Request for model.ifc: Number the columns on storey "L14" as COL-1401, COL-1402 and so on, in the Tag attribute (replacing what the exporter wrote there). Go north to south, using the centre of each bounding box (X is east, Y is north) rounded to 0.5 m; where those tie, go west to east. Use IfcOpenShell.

First a look at what the model holds.

```python
import ifcopenshell
import ifcopenshell.util.element
import ifcopenshell.util.placement

model = ifcopenshell.open("model.ifc")
print(model.schema)
storey = next(s for s in model.by_type("IfcBuildingStorey") if s.Name == "L14")
columns = [e for e in ifcopenshell.util.element.get_decomposition(storey) if e.is_a("IfcColumn")]
for e in sorted(columns, key=lambda e: e.id()):
    origin = ifcopenshell.util.placement.get_local_placement(e.ObjectPlacement)[:3, 3]
    print(e.id(), e.Tag, e.Name, origin.round(2) + 0.0, sep=" | ")
```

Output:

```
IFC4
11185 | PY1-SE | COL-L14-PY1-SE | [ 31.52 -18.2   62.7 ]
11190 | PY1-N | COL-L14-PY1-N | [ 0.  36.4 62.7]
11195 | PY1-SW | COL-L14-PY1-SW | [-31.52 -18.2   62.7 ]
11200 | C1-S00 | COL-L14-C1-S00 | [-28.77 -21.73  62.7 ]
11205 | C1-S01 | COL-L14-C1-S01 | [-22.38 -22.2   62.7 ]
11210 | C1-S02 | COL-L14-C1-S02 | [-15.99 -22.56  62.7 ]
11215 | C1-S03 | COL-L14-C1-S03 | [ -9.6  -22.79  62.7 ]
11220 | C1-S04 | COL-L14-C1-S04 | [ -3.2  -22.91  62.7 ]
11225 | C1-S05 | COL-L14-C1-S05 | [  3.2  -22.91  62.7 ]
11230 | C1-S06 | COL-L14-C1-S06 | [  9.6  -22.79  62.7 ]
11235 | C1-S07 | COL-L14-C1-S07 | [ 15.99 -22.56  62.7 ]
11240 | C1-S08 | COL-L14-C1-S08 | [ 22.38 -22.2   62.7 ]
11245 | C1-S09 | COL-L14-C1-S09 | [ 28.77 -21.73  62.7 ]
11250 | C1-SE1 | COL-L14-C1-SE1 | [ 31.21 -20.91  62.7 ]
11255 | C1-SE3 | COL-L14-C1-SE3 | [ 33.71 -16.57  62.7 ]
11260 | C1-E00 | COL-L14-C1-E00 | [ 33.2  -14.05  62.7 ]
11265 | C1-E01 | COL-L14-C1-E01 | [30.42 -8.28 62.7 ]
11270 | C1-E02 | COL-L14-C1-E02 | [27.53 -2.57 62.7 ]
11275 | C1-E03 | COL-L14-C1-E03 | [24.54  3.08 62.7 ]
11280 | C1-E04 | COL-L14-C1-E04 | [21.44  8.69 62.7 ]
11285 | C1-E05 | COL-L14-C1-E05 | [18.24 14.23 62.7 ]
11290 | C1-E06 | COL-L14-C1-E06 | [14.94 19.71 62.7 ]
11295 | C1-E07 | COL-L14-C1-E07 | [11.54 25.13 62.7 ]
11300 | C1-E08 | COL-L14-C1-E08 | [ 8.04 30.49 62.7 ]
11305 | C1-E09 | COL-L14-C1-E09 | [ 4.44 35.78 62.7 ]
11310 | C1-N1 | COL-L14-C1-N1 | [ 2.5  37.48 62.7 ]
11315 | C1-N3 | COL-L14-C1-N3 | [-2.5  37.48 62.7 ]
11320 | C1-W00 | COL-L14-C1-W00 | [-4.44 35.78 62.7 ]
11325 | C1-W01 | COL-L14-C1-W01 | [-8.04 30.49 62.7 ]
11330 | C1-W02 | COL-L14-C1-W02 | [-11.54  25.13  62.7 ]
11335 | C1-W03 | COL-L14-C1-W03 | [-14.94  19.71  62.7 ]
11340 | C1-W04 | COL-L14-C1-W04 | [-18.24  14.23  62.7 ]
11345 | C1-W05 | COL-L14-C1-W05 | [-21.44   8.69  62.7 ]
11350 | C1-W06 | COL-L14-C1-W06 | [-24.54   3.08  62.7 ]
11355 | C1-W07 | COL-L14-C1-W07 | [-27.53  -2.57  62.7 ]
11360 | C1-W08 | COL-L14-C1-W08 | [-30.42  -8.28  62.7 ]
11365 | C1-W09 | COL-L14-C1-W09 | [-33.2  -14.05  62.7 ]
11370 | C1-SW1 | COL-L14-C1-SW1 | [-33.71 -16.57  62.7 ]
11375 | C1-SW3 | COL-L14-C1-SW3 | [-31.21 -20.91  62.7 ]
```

```python
import ifcopenshell
import ifcopenshell.geom
import ifcopenshell.util.element
import ifcopenshell.util.shape

model = ifcopenshell.open("model.ifc")
settings = ifcopenshell.geom.settings()
settings.set("use-world-coords", True)


def centre(element):
    shape = ifcopenshell.geom.create_shape(settings, element)
    return ifcopenshell.util.shape.get_bbox_centroid(shape.geometry)


storey = next(s for s in model.by_type("IfcBuildingStorey") if s.Name == "L14")
columns = [e for e in ifcopenshell.util.element.get_decomposition(storey) if e.is_a("IfcColumn")]

# Insertion points can sit at a corner or the storey origin, so sort by the geometry (in metres).
centres = {e: centre(e) for e in columns}
columns.sort(key=lambda e: (-round(centres[e][1] / 0.5), centres[e][0]))

for i, e in enumerate(columns, start=1):
    number = f"COL-14{i:02d}"
    e.Tag = number
    print(e.id(), number)

model.write("model-out.ifc")
```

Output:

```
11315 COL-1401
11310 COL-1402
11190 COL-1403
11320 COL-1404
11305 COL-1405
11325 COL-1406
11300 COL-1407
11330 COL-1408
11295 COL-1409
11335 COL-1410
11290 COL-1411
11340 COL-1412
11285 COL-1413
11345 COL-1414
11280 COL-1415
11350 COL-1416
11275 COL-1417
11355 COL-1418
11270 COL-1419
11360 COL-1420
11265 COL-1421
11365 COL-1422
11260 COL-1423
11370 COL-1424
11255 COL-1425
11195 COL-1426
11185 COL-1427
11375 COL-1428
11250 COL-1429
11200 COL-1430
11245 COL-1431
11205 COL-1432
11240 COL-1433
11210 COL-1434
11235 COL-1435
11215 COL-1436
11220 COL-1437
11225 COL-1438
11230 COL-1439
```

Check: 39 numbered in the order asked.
